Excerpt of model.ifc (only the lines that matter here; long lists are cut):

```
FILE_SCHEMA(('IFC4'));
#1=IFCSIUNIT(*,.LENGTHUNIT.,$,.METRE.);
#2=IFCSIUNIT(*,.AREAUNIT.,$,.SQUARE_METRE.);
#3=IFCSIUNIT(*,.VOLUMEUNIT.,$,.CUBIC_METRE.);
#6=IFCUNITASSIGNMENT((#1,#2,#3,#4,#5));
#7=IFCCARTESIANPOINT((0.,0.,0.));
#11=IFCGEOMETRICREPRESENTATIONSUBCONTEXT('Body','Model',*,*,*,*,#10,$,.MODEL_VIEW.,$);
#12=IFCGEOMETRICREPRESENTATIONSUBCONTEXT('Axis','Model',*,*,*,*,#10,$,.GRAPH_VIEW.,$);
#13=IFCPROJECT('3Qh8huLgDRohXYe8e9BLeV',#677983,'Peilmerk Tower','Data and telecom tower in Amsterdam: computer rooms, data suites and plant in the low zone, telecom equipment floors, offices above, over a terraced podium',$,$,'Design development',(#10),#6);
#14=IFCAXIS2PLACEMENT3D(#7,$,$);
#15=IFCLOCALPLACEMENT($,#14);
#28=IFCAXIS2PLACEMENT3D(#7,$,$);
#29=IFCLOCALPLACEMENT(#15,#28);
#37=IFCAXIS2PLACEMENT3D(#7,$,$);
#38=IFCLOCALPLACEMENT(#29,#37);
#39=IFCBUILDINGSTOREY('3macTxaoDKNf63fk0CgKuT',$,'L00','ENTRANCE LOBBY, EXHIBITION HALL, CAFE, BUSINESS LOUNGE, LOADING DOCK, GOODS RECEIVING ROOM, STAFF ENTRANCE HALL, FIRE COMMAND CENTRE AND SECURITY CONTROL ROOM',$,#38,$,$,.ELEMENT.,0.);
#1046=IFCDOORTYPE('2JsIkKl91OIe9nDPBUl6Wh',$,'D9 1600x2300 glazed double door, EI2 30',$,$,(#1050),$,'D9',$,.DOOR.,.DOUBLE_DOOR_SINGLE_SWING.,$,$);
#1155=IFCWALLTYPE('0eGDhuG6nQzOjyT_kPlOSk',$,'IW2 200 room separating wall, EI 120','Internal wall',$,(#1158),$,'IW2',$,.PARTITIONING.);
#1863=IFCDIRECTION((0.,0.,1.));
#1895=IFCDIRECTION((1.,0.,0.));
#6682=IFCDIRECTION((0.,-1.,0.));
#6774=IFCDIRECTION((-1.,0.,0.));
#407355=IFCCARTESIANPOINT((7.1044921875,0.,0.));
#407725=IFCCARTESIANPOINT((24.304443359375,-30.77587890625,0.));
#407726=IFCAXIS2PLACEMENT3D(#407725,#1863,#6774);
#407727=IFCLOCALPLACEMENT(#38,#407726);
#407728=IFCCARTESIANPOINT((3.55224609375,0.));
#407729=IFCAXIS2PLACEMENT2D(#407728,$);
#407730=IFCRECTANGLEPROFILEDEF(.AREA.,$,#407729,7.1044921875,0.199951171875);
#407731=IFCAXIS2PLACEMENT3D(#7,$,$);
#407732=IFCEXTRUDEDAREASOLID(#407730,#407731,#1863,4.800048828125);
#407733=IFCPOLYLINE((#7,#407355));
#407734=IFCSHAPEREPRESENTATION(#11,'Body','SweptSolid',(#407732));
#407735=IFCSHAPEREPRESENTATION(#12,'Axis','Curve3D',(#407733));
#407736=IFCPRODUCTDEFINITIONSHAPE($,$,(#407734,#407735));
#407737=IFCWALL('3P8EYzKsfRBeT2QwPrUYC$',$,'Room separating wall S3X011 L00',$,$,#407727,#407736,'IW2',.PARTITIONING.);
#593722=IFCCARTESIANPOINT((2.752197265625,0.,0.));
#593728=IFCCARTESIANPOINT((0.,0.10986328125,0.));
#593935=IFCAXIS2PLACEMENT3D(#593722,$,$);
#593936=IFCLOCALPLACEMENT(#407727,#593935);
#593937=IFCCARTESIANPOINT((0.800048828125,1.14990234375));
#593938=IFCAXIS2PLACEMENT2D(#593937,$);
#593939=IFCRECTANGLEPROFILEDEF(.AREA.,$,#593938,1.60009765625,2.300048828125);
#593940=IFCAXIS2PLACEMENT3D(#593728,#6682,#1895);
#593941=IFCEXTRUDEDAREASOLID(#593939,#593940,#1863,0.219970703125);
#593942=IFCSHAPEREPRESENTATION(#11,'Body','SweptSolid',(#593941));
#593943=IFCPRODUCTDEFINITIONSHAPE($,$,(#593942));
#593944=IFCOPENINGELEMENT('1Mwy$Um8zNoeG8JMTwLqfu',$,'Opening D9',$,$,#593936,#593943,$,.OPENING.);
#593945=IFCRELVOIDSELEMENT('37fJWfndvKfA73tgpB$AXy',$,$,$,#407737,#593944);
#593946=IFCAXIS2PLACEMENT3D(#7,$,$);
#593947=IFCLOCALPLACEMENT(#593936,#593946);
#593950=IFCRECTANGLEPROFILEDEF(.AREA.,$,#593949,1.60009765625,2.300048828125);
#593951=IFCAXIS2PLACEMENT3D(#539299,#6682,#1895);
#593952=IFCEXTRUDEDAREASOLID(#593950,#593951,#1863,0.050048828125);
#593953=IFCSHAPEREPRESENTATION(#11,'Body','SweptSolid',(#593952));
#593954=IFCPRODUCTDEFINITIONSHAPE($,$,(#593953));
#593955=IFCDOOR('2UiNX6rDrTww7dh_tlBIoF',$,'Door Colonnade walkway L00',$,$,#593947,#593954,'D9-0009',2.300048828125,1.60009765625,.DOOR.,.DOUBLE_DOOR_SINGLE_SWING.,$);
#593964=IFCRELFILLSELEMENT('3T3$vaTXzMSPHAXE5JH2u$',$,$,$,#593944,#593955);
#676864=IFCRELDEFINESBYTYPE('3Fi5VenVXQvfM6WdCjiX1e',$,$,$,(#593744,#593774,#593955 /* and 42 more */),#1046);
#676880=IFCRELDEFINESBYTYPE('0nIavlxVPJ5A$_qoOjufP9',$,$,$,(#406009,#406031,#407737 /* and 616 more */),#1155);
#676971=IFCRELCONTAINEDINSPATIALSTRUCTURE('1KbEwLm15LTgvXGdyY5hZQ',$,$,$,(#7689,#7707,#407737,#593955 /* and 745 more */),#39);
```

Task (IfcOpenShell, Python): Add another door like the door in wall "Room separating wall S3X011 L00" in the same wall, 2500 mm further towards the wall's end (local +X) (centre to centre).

```python
import ifcopenshell
import ifcopenshell.api.feature
import ifcopenshell.api.geometry
import ifcopenshell.api.root
import ifcopenshell.geom
import ifcopenshell.util.element
import ifcopenshell.util.placement
import ifcopenshell.util.shape
import ifcopenshell.util.unit

model = ifcopenshell.open("model.ifc")
unit_scale = ifcopenshell.util.unit.calculate_unit_scale(model)
settings = ifcopenshell.geom.settings()


def volume(element):
    """Net volume in cubic metres, openings subtracted."""
    shape = ifcopenshell.geom.create_shape(settings, element)
    return ifcopenshell.util.shape.get_volume(shape.geometry)


door = model.by_guid("2UiNX6rDrTww7dh_tlBIoF")
opening = door.FillsVoids[0].RelatingOpeningElement
wall = opening.VoidsElements[0].RelatingBuildingElement
before = volume(wall)
shift = ifcopenshell.util.placement.get_local_placement(wall.ObjectPlacement)[:3, 0] * 2.5 / unit_scale

# copy_class copies the void relationship, type, container and properties, but no geometry.
new_opening = ifcopenshell.api.root.copy_class(model, product=opening)
new_opening.Representation = ifcopenshell.util.element.copy_deep(
    model, opening.Representation, exclude=["IfcGeometricRepresentationContext", "IfcRepresentationMap"]
)
new_door = ifcopenshell.api.root.copy_class(model, product=door)
new_door.Representation = ifcopenshell.util.element.copy_deep(
    model, door.Representation, exclude=["IfcGeometricRepresentationContext", "IfcRepresentationMap"]
)
new_door.Tag = None
ifcopenshell.api.feature.add_filling(model, opening=new_opening, element=new_door)

for old, new in ((opening, new_opening), (door, new_door)):
    matrix = ifcopenshell.util.placement.get_local_placement(old.ObjectPlacement)
    matrix[:3, 3] += shift
    ifcopenshell.api.geometry.edit_object_placement(model, product=new, matrix=matrix, is_si=False)

after = volume(wall)

print(f"wall volume {before:.3f} -> {after:.3f} m3")

model.write("model_updated.ifc")
```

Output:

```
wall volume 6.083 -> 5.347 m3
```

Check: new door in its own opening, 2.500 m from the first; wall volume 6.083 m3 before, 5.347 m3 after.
